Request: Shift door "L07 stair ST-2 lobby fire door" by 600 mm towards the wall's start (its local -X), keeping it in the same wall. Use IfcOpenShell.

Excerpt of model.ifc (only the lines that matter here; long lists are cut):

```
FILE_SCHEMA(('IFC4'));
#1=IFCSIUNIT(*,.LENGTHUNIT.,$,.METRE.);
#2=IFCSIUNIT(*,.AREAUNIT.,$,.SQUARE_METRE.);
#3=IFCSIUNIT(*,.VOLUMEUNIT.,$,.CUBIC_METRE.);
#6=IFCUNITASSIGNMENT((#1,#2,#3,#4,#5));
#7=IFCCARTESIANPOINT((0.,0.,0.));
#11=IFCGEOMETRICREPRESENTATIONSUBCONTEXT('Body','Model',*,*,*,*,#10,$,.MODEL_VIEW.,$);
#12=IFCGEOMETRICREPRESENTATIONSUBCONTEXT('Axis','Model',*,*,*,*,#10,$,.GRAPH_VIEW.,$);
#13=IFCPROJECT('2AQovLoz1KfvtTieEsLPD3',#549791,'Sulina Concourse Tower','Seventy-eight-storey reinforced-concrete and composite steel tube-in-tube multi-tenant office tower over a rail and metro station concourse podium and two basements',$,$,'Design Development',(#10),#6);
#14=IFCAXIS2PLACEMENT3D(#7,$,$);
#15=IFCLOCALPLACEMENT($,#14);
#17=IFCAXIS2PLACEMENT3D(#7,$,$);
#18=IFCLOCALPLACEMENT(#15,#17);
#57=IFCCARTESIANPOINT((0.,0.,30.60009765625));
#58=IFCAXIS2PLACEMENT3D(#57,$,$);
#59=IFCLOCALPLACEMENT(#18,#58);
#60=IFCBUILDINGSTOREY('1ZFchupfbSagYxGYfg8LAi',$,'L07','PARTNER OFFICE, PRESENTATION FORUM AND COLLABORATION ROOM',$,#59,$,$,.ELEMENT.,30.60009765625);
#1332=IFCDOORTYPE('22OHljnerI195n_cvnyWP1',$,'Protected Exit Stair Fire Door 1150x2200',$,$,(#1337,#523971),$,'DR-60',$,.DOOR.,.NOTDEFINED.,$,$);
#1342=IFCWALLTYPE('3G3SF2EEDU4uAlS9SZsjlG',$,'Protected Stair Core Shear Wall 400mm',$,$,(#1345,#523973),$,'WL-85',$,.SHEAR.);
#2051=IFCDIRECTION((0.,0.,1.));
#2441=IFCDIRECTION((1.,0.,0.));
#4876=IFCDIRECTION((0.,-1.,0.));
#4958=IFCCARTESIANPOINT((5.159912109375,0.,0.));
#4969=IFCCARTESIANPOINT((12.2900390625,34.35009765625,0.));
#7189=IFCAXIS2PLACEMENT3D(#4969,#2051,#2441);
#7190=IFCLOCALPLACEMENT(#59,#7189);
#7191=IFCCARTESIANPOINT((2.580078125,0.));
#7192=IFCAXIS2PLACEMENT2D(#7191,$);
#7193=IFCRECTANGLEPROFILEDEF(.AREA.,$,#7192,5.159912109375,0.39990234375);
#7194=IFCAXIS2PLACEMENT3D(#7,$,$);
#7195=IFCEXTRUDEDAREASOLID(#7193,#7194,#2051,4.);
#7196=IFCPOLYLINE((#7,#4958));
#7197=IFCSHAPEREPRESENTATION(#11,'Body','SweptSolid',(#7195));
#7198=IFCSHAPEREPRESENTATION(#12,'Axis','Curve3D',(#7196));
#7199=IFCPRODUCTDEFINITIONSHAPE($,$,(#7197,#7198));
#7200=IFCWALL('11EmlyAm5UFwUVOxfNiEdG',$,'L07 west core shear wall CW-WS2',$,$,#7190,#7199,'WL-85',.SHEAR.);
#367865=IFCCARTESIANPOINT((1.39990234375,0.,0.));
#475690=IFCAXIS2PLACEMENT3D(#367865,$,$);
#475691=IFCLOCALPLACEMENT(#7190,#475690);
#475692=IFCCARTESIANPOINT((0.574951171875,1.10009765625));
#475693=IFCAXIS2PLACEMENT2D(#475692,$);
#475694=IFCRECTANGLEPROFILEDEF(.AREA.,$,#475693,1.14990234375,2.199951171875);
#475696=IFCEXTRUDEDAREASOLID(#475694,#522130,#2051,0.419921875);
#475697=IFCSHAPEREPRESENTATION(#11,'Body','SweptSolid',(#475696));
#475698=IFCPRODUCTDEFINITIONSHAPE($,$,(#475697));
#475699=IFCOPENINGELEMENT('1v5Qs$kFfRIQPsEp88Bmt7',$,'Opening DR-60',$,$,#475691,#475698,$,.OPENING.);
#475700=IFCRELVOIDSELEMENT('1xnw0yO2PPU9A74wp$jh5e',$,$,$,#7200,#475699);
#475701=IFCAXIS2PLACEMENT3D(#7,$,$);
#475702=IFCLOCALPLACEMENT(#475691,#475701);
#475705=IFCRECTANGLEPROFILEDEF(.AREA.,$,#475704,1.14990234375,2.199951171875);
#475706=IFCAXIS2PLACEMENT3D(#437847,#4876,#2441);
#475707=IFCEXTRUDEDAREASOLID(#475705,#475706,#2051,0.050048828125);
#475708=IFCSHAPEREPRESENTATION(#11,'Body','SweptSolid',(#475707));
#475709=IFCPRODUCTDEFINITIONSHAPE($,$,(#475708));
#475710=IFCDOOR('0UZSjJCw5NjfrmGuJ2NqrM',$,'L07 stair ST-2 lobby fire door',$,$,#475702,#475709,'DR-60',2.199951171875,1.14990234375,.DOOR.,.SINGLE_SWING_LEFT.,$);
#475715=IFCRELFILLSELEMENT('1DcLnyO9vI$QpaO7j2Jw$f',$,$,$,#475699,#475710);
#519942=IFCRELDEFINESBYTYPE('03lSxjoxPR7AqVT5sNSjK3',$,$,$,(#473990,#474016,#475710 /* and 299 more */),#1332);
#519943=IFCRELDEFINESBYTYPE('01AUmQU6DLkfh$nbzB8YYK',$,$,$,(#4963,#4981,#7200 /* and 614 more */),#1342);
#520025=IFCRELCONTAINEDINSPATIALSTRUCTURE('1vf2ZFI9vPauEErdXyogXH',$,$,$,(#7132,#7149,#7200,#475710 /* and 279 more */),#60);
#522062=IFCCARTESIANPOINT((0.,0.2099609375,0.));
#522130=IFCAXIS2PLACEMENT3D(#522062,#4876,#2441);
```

```python
import ifcopenshell
import ifcopenshell.api.geometry
import ifcopenshell.util.placement
import ifcopenshell.util.unit

model = ifcopenshell.open("model.ifc")
unit_scale = ifcopenshell.util.unit.calculate_unit_scale(model)

door = model.by_id(475710)
opening = door.FillsVoids[0].RelatingOpeningElement
wall = opening.VoidsElements[0].RelatingBuildingElement

wall_matrix = ifcopenshell.util.placement.get_local_placement(wall.ObjectPlacement)
shift = wall_matrix[:3, 0] * -0.6 / unit_scale
before = ifcopenshell.util.placement.get_local_placement(door.ObjectPlacement)[:3, 3].copy()

# The door is placed relative to its opening, so it follows when the opening moves.
matrix = ifcopenshell.util.placement.get_local_placement(opening.ObjectPlacement)
matrix[:3, 3] += shift
ifcopenshell.api.geometry.edit_object_placement(
    model, product=opening, matrix=matrix, is_si=False, should_transform_children=True
)

after = ifcopenshell.util.placement.get_local_placement(door.ObjectPlacement)[:3, 3]
print("door moved by", (after - before).round(3) + 0.0)

model.write("model-out.ifc")
```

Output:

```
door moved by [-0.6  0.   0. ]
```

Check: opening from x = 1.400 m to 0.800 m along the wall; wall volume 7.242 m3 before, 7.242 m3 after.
